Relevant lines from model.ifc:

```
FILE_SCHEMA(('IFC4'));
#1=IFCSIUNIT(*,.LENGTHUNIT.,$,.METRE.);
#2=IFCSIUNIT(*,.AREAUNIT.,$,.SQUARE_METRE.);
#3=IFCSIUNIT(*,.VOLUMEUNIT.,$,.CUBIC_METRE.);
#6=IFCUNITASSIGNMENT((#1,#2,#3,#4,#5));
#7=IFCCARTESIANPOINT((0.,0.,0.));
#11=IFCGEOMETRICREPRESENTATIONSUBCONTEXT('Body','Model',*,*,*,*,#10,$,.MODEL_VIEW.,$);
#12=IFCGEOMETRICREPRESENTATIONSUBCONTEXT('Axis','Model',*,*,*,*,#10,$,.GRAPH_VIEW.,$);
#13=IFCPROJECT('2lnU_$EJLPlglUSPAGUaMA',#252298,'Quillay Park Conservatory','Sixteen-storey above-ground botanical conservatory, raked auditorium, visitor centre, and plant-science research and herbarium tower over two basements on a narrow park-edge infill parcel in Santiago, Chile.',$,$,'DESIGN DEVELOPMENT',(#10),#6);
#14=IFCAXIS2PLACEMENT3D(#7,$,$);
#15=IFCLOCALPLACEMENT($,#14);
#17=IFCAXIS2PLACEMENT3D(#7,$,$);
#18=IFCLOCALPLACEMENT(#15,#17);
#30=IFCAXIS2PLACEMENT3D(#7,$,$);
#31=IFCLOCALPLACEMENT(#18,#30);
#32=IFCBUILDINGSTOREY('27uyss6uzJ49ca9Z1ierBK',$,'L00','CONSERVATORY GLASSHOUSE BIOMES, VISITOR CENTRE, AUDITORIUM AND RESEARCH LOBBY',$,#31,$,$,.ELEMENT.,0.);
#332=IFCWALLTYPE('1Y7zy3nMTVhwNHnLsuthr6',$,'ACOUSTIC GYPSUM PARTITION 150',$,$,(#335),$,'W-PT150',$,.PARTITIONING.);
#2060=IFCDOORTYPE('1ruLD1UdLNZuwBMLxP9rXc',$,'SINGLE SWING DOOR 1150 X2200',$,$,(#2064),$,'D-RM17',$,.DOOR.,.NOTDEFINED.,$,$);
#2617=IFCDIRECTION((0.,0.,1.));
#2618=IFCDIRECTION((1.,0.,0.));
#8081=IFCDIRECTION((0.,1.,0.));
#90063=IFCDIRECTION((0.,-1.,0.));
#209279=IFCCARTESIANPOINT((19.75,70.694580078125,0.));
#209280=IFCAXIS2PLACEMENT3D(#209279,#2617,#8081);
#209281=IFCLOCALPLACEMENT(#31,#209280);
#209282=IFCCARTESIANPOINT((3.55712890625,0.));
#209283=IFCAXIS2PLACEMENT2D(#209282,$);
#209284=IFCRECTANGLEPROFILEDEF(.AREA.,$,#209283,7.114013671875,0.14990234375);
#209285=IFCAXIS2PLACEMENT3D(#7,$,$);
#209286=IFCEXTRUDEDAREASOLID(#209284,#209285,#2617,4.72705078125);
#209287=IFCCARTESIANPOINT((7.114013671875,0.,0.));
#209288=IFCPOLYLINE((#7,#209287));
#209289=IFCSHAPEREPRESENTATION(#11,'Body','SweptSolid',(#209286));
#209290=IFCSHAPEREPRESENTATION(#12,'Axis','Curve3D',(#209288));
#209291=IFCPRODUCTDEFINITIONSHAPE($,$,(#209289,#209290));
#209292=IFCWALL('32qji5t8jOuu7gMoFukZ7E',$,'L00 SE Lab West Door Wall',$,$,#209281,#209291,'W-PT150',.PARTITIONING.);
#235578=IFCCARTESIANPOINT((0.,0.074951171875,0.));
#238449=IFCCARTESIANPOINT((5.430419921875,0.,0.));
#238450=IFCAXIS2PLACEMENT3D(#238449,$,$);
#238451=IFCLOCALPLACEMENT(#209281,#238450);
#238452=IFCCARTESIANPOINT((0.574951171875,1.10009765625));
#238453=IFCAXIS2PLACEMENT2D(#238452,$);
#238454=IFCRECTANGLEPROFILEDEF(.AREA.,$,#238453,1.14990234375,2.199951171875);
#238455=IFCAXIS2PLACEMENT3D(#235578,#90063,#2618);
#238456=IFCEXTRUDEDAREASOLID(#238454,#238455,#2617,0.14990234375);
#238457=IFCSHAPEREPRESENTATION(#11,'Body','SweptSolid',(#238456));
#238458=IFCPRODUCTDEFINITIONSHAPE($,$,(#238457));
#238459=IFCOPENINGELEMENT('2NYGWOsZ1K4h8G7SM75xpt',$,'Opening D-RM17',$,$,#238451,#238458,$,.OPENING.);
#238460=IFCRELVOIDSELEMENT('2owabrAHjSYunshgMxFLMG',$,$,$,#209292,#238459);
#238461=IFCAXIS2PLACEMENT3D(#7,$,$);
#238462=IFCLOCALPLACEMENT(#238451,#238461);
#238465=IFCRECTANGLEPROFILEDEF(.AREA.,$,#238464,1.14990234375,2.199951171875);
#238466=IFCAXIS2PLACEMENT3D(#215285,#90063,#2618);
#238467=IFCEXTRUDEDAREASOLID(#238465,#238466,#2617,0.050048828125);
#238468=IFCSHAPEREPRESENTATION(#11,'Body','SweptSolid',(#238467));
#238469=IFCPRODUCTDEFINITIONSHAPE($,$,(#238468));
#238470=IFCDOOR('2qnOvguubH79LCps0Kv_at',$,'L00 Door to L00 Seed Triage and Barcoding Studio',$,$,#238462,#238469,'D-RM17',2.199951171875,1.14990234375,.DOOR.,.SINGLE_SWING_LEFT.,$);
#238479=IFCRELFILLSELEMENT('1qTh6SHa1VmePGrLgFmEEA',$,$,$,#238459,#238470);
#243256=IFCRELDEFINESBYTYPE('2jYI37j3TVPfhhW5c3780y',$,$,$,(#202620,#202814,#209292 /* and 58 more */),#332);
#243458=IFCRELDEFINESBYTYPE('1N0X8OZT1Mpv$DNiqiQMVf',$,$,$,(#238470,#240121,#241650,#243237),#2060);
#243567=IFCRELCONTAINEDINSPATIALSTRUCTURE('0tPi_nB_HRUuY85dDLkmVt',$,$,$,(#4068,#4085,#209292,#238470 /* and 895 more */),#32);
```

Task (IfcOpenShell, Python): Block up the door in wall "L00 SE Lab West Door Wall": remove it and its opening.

```python
import ifcopenshell
import ifcopenshell.api.feature
import ifcopenshell.api.root
import ifcopenshell.geom
import ifcopenshell.util.shape

model = ifcopenshell.open("model.ifc")
settings = ifcopenshell.geom.settings()


def volume(element):
    """Net volume in cubic metres, openings subtracted."""
    shape = ifcopenshell.geom.create_shape(settings, element)
    return ifcopenshell.util.shape.get_volume(shape.geometry)


door = model.by_guid("2qnOvguubH79LCps0Kv_at")
opening = door.FillsVoids[0].RelatingOpeningElement
wall = opening.VoidsElements[0].RelatingBuildingElement
before = volume(wall)

ifcopenshell.api.root.remove_product(model, product=door)
ifcopenshell.api.feature.remove_feature(model, feature=opening)

after = volume(wall)

print(f"wall volume {before:.3f} -> {after:.3f} m3")

model.write("model_updated.ifc")
```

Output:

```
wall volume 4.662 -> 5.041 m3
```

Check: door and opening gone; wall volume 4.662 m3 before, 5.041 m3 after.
